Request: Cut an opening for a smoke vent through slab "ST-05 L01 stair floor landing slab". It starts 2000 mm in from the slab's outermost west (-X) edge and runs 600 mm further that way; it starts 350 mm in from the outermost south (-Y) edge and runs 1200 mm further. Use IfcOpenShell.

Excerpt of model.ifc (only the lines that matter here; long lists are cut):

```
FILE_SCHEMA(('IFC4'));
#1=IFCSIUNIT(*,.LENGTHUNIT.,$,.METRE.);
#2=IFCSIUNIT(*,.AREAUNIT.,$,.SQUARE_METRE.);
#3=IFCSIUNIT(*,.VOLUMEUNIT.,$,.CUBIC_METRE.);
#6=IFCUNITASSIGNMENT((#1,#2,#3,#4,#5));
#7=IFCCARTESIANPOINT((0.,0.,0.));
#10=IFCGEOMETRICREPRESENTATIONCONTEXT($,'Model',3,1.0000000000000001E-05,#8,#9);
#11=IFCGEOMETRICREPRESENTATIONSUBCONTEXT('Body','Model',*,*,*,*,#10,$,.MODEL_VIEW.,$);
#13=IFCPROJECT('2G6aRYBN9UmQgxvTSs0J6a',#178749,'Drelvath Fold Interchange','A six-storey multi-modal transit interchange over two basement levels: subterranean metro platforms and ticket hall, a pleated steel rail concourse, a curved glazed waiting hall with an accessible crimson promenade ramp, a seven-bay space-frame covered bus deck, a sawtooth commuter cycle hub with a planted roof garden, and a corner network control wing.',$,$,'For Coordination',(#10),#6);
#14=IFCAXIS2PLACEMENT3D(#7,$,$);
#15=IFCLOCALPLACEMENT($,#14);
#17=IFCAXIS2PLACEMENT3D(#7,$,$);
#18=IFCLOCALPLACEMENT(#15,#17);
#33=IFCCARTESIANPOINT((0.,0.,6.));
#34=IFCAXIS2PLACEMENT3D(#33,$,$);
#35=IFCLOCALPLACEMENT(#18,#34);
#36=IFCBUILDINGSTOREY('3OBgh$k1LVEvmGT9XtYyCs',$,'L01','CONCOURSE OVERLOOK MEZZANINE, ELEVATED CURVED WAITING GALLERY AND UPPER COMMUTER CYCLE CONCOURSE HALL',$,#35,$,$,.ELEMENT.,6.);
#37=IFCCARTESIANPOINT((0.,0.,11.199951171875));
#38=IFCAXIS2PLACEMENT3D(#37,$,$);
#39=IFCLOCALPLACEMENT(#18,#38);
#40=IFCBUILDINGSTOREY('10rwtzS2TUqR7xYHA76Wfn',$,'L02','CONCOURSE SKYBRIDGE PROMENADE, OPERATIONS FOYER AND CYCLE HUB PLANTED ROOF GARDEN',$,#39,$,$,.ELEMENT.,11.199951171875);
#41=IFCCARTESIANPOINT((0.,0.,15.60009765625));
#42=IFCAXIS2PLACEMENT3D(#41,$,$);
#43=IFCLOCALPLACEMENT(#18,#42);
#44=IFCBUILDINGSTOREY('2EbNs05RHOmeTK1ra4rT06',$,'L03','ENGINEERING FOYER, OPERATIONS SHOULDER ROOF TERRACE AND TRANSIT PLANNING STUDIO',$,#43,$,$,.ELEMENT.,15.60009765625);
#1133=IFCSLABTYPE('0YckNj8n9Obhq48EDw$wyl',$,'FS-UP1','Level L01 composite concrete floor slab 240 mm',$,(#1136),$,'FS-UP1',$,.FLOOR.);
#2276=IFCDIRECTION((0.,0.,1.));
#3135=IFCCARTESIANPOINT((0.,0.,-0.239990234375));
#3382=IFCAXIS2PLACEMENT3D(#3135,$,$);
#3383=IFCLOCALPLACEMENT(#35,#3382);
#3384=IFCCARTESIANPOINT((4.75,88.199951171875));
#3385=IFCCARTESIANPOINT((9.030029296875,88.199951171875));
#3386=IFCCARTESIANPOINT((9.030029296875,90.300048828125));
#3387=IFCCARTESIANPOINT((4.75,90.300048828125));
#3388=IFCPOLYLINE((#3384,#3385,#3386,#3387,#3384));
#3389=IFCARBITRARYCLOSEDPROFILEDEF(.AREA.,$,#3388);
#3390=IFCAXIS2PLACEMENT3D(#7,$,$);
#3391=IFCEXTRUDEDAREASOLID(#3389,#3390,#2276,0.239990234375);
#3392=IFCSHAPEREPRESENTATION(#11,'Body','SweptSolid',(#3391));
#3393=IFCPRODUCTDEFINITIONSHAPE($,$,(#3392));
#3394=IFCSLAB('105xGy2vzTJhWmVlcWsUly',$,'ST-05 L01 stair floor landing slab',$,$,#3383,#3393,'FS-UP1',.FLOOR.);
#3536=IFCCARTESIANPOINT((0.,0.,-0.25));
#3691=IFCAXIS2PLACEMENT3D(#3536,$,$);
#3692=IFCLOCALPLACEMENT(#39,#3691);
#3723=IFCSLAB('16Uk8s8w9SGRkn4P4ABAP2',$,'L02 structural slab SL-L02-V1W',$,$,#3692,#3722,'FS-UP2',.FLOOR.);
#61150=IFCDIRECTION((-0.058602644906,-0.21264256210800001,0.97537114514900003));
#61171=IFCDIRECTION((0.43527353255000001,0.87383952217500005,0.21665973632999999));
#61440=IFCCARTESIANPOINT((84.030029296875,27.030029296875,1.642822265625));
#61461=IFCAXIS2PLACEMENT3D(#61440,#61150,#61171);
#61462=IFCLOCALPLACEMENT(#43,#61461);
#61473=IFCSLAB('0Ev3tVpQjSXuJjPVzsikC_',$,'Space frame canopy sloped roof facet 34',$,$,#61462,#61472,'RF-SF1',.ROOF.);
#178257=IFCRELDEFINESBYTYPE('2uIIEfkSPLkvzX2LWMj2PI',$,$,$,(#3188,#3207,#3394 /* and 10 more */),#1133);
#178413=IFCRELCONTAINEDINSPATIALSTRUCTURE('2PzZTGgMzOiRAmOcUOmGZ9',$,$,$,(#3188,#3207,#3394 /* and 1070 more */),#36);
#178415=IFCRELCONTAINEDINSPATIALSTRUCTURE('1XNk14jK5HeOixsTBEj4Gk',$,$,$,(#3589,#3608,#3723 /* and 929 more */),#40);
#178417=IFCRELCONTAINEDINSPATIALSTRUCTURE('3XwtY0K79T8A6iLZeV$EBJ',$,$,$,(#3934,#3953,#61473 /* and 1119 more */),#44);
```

```python
import numpy as np
import ifcopenshell
import ifcopenshell.api.feature
import ifcopenshell.api.geometry
import ifcopenshell.api.root
import ifcopenshell.geom
import ifcopenshell.util.placement
import ifcopenshell.util.representation
import ifcopenshell.util.shape
import ifcopenshell.util.unit

model = ifcopenshell.open("model.ifc")
unit_scale = ifcopenshell.util.unit.calculate_unit_scale(model)
settings = ifcopenshell.geom.settings()


def volume(element):
    """Net volume in cubic metres, openings subtracted."""
    shape = ifcopenshell.geom.create_shape(settings, element)
    return ifcopenshell.util.shape.get_volume(shape.geometry)


slab = model.by_guid("105xGy2vzTJhWmVlcWsUly")
before = volume(slab)

# Extent in the slab's own axes, in metres. The edges named are its -X and -Y sides.
slab_shape = ifcopenshell.geom.create_shape(settings, slab)
vertices = ifcopenshell.util.shape.get_vertices(slab_shape.geometry)
x_min, y_min, bottom = vertices.min(axis=0)
top = vertices[:, 2].max()

opening = ifcopenshell.api.root.create_entity(model, ifc_class="IfcOpeningElement", name="Smoke vent opening", predefined_type="OPENING")
context = ifcopenshell.util.representation.get_context(model, "Model", "Body", "MODEL_VIEW")
width, depth = 0.6, 1.2
outline = [(0.0, 0.0), (width, 0.0), (width, depth), (0.0, depth), (0.0, 0.0)]
# Overshoot both faces by 50 mm so the cut is clean.
shape = ifcopenshell.api.geometry.add_slab_representation(
    model, context=context, depth=top - bottom + 0.1, polyline=outline
)
ifcopenshell.api.geometry.assign_representation(model, product=opening, representation=shape)

matrix = ifcopenshell.util.placement.get_local_placement(slab.ObjectPlacement)
matrix[:, 3] = matrix @ np.append(np.array([x_min + 2, y_min + 0.35, bottom - 0.05]) / unit_scale, 1.0)
ifcopenshell.api.geometry.edit_object_placement(model, product=opening, matrix=matrix, is_si=False)
ifcopenshell.api.feature.add_feature(model, feature=opening, element=slab)

after = volume(slab)

print(f"slab volume {before:.3f} -> {after:.3f} m3")

model.write("model-out.ifc")
```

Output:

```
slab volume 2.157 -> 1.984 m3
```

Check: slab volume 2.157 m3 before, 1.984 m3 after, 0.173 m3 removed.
